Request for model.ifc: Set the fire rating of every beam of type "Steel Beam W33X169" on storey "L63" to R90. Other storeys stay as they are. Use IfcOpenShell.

First a look at what the model holds.

```python
import ifcopenshell
import ifcopenshell.util.element

model = ifcopenshell.open("model.ifc")
print(model.schema)
storey = next(s for s in model.by_type("IfcBuildingStorey") if s.Name == "L63")
beams = [e for e in ifcopenshell.util.element.get_decomposition(storey) if e.is_a("IfcBeam")]
seen = {}
for e in beams:
    element_type = ifcopenshell.util.element.get_type(e)
    key = (element_type.Name if element_type != e and element_type else None, ifcopenshell.util.element.get_pset(e, "Pset_BeamCommon", "FireRating"))
    seen[key] = seen.get(key, 0) + 1
for (name, value), count in sorted(seen.items(), key=str):
    print(count, "x", name, "|", value)
```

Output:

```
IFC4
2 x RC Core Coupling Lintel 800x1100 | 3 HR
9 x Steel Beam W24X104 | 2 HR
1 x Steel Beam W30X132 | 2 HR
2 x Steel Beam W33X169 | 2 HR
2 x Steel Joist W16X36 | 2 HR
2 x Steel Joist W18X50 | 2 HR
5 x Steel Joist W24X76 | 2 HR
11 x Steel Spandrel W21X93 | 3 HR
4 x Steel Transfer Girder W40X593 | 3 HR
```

```python
import ifcopenshell
import ifcopenshell.api.pset
import ifcopenshell.util.element

model = ifcopenshell.open("model.ifc")

storey = next(s for s in model.by_type("IfcBuildingStorey") if s.Name == "L63")
beams = [e for e in ifcopenshell.util.element.get_decomposition(storey) if e.is_a("IfcBeam")]

count = 0
for e in beams:
    element_type = ifcopenshell.util.element.get_type(e)
    if element_type in (None, e) or element_type.Name != "Steel Beam W33X169":
        continue
    found = ifcopenshell.util.element.get_pset(e, "Pset_BeamCommon", should_inherit=False)
    if found:
        pset = model.by_id(found["id"])
        if len(ifcopenshell.util.element.get_elements_by_pset(pset)) > 1:
            pset = ifcopenshell.api.pset.unshare_pset(model, products=[e], pset=pset)[0]
    else:
        pset = ifcopenshell.api.pset.add_pset(model, product=e, name="Pset_BeamCommon")
    ifcopenshell.api.pset.edit_pset(model, pset=pset, properties={"FireRating": "R90"})
    count += 1

print(count, "beams updated")

model.write("model_updated.ifc")
```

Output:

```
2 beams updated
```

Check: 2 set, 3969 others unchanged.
